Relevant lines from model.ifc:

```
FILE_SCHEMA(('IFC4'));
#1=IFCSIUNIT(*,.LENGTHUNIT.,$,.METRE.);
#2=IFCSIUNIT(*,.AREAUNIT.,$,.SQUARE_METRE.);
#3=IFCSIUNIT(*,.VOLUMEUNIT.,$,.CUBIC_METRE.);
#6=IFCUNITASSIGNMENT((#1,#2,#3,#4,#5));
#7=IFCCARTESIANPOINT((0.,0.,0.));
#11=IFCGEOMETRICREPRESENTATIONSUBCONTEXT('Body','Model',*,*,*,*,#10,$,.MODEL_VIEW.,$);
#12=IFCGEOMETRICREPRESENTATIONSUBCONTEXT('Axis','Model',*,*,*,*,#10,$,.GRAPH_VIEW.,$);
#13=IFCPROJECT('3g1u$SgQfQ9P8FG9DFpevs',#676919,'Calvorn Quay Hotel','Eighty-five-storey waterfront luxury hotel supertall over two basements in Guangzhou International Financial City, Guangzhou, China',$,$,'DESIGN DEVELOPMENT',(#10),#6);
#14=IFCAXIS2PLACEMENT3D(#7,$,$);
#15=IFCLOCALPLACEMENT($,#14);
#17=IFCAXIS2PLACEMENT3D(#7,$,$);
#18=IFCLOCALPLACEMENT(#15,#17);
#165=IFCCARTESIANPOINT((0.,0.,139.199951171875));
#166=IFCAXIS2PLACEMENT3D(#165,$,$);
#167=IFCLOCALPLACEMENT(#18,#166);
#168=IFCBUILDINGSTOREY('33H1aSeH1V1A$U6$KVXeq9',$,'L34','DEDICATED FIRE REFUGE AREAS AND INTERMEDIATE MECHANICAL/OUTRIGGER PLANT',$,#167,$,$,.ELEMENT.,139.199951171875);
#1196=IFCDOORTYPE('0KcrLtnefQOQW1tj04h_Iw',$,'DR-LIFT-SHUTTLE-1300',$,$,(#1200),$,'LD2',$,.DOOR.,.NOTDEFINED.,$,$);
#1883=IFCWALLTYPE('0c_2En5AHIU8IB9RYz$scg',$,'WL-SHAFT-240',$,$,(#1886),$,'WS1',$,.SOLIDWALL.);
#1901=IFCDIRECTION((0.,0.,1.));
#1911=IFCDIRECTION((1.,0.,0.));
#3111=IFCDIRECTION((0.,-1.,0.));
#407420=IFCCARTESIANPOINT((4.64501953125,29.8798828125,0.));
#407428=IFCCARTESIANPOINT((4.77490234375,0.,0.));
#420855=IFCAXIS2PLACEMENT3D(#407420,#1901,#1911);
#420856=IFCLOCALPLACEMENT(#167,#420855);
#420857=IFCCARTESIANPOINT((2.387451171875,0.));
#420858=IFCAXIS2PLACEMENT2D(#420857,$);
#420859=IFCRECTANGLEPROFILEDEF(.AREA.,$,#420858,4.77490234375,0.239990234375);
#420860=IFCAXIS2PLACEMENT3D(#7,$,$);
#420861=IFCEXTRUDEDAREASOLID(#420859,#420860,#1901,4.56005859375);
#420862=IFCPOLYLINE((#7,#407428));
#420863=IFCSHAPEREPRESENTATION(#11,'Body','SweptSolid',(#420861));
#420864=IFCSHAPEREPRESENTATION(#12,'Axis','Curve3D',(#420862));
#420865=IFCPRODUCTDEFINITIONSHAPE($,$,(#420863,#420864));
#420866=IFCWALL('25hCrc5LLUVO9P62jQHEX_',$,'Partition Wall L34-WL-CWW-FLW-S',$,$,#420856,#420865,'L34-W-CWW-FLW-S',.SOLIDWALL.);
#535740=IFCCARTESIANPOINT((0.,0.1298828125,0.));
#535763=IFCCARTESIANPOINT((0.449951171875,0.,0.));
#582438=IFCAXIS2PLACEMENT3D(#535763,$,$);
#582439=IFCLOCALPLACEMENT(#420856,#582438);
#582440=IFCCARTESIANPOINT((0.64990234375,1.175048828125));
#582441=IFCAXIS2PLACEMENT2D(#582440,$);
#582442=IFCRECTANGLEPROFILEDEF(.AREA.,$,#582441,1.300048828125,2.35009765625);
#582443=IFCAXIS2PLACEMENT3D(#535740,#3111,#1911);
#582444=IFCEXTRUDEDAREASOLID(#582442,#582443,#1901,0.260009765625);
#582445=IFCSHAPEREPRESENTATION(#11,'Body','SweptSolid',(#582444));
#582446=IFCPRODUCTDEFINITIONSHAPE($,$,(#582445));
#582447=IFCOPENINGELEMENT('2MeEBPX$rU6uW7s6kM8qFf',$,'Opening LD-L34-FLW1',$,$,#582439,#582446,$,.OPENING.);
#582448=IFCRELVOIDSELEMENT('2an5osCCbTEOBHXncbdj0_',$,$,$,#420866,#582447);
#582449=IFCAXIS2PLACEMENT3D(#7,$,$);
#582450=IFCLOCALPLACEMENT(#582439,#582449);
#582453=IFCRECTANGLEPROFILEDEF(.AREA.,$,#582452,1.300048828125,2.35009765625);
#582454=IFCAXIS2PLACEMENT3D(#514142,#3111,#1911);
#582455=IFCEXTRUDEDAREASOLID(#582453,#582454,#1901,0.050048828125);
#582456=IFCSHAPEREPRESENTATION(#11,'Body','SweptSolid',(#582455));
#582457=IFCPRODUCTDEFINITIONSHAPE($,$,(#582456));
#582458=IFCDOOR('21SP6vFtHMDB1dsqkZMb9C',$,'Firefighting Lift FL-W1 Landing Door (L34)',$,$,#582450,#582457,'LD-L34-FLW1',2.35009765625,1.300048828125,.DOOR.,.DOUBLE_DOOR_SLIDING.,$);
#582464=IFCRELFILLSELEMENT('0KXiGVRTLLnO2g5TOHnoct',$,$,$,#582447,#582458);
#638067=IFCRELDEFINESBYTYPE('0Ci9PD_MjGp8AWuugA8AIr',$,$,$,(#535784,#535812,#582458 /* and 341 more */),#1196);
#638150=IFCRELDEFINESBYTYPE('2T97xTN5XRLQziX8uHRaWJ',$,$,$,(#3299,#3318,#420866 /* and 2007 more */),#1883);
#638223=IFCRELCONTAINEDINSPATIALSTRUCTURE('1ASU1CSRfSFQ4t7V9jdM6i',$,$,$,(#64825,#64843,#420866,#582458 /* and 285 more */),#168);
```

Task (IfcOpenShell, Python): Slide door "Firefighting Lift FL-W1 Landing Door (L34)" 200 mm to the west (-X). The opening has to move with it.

```python
import ifcopenshell
import ifcopenshell.api.geometry
import ifcopenshell.util.placement

model = ifcopenshell.open("model.ifc")

door = model.by_guid("21SP6vFtHMDB1dsqkZMb9C")
opening = door.FillsVoids[0].RelatingOpeningElement
wall = opening.VoidsElements[0].RelatingBuildingElement

wall_matrix = ifcopenshell.util.placement.get_local_placement(wall.ObjectPlacement)
shift = wall_matrix[:3, 0] * -0.2
before = ifcopenshell.util.placement.get_local_placement(door.ObjectPlacement)[:3, 3].copy()

# The door is placed relative to its opening, so it follows when the opening moves.
matrix = ifcopenshell.util.placement.get_local_placement(opening.ObjectPlacement)
matrix[:3, 3] += shift
ifcopenshell.api.geometry.edit_object_placement(
    model, product=opening, matrix=matrix, is_si=False, should_transform_children=True
)

after = ifcopenshell.util.placement.get_local_placement(door.ObjectPlacement)[:3, 3]
print("door moved by", (after - before).round(3) + 0.0)

model.write("model_updated.ifc")
```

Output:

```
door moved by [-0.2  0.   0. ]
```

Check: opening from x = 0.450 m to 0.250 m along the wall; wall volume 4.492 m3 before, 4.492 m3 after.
